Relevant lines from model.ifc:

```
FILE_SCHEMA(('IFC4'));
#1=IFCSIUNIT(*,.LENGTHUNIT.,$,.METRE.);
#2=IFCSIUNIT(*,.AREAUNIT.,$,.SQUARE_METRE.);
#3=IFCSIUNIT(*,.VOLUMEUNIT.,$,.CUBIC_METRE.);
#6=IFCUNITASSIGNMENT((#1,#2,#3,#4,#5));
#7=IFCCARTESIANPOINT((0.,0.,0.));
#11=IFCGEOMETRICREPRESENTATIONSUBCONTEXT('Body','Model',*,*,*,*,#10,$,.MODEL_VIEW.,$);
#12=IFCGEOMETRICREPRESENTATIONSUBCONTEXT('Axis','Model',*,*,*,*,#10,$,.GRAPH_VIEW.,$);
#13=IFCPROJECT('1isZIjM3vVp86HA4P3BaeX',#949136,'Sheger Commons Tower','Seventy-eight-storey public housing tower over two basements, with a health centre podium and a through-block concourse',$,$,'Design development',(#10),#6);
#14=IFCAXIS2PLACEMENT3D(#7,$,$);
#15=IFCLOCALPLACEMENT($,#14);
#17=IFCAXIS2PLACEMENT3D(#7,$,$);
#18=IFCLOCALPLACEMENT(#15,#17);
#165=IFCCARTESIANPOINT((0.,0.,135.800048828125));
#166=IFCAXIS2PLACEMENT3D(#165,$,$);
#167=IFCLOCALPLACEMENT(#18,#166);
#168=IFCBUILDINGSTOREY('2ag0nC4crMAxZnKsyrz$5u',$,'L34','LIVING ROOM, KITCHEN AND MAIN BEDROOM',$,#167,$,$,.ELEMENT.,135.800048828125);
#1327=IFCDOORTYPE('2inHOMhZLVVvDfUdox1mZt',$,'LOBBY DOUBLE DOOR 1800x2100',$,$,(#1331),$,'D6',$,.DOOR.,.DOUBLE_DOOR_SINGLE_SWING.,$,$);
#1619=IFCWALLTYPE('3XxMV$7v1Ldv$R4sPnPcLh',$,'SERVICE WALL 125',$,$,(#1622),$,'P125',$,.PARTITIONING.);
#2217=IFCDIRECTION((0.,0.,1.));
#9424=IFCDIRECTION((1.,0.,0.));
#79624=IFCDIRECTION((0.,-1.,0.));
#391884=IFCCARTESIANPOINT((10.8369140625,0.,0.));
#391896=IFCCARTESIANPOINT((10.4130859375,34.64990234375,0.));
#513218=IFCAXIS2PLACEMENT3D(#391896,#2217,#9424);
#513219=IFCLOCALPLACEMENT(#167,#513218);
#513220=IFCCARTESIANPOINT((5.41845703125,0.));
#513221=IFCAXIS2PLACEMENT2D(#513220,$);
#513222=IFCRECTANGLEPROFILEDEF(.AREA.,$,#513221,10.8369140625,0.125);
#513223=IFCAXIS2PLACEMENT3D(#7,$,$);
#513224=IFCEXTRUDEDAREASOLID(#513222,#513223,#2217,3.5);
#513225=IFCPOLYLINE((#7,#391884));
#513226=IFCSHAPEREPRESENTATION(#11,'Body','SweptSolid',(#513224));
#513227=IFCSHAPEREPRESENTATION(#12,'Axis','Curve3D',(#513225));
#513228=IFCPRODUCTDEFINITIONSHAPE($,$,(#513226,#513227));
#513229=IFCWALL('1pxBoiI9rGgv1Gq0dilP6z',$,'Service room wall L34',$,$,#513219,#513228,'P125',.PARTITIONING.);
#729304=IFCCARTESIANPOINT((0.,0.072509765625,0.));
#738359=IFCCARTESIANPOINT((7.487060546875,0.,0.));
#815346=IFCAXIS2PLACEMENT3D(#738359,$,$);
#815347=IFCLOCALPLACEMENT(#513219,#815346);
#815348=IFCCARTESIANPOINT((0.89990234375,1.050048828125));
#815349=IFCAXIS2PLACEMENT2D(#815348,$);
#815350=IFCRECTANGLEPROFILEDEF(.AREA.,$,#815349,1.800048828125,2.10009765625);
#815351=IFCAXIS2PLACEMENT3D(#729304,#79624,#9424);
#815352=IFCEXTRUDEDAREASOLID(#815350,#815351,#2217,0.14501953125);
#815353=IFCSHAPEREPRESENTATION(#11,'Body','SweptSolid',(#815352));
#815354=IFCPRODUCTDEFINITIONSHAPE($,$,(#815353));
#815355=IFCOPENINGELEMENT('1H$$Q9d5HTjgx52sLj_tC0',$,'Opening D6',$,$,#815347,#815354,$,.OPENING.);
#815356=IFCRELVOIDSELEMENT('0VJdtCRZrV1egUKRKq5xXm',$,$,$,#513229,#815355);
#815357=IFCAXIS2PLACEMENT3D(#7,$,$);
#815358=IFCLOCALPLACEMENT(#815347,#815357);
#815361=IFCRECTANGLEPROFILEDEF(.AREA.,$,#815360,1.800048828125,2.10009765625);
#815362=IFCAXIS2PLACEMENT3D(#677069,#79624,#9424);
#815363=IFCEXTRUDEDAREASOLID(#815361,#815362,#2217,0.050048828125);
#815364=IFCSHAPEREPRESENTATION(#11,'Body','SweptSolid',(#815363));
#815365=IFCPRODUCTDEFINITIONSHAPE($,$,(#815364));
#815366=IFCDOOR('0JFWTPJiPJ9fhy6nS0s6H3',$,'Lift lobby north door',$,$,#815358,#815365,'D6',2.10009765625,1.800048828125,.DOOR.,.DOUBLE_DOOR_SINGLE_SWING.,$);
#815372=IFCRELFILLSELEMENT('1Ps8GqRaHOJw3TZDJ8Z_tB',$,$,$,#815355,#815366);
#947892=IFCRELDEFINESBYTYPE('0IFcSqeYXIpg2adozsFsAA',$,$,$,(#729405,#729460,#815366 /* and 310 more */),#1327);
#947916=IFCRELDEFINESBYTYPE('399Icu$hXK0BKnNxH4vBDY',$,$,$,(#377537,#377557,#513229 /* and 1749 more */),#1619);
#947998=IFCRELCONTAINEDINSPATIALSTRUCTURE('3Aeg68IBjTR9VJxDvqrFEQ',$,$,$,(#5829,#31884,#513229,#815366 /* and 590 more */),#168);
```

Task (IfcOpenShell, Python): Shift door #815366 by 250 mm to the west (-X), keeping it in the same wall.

```python
import ifcopenshell
import ifcopenshell.api.geometry
import ifcopenshell.util.placement

model = ifcopenshell.open("model.ifc")

door = model.by_id(815366)
opening = door.FillsVoids[0].RelatingOpeningElement
wall = opening.VoidsElements[0].RelatingBuildingElement

wall_matrix = ifcopenshell.util.placement.get_local_placement(wall.ObjectPlacement)
shift = wall_matrix[:3, 0] * -0.25
before = ifcopenshell.util.placement.get_local_placement(door.ObjectPlacement)[:3, 3].copy()

# The door is placed relative to its opening, so it follows when the opening moves.
matrix = ifcopenshell.util.placement.get_local_placement(opening.ObjectPlacement)
matrix[:3, 3] += shift
ifcopenshell.api.geometry.edit_object_placement(
    model, product=opening, matrix=matrix, is_si=False, should_transform_children=True
)

after = ifcopenshell.util.placement.get_local_placement(door.ObjectPlacement)[:3, 3]
print("door moved by", (after - before).round(3) + 0.0)

model.write("model-out.ifc")
```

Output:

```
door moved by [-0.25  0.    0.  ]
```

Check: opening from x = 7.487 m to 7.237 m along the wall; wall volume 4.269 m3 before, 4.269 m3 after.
